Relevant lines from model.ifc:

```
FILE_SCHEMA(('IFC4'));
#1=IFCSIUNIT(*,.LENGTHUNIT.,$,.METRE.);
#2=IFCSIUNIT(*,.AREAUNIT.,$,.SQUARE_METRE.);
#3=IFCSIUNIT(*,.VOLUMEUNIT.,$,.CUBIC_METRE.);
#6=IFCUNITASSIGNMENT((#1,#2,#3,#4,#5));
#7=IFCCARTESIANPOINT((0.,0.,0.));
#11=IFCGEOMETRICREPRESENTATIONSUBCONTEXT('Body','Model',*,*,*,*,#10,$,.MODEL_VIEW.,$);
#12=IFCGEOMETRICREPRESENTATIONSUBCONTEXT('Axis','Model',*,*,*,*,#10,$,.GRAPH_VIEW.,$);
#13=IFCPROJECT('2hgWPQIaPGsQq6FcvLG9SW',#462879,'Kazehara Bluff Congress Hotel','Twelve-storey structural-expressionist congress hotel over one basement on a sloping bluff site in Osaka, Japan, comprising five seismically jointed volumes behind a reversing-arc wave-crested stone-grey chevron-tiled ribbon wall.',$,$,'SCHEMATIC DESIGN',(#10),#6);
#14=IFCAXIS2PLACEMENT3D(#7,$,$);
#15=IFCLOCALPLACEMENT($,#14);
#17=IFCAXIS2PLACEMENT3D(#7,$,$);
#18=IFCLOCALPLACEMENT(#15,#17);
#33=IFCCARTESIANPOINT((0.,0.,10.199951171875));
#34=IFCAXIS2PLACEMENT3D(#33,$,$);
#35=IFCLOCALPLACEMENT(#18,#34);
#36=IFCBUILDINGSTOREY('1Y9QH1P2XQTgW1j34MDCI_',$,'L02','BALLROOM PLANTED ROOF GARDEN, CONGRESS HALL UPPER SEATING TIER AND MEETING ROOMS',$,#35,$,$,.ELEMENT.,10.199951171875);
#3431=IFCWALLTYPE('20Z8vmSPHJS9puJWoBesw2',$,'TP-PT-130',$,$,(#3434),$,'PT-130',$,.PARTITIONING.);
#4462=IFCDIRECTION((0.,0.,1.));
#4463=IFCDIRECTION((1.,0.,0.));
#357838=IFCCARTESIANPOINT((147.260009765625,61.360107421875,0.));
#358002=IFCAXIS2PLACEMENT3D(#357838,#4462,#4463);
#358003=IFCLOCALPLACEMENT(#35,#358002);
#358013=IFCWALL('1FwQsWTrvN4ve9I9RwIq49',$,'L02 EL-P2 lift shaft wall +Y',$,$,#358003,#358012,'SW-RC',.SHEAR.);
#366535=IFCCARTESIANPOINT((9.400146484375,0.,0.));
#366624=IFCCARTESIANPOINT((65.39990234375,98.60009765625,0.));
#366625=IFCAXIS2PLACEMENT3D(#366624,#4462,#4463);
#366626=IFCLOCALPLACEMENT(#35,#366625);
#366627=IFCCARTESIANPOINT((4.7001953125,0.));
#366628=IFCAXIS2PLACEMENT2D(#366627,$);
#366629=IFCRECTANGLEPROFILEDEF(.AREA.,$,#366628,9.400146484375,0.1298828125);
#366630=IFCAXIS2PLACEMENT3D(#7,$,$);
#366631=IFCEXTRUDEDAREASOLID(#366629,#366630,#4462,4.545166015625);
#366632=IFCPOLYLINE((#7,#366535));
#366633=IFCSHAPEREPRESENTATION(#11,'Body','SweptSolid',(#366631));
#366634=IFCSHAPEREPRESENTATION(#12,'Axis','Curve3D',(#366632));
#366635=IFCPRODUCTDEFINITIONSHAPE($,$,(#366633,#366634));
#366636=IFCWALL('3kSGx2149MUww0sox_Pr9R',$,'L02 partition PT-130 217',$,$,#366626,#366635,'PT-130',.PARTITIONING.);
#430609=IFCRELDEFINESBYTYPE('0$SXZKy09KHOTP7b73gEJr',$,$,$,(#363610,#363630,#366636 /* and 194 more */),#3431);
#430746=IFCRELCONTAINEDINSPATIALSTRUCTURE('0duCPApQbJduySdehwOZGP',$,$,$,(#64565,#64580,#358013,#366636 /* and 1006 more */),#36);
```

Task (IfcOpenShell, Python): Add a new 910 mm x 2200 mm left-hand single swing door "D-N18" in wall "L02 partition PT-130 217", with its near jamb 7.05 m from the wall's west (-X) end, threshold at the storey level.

```python
import numpy as np
import ifcopenshell
import ifcopenshell.api.feature
import ifcopenshell.api.geometry
import ifcopenshell.api.root
import ifcopenshell.api.spatial
import ifcopenshell.geom
import ifcopenshell.util.element
import ifcopenshell.util.placement
import ifcopenshell.util.representation
import ifcopenshell.util.shape
import ifcopenshell.util.unit

model = ifcopenshell.open("model.ifc")
unit_scale = ifcopenshell.util.unit.calculate_unit_scale(model)
settings = ifcopenshell.geom.settings()


def volume(element):
    """Net volume in cubic metres, openings subtracted."""
    shape = ifcopenshell.geom.create_shape(settings, element)
    return ifcopenshell.util.shape.get_volume(shape.geometry)


wall = model.by_id(366636)
storey = ifcopenshell.util.element.get_container(wall, ifc_class="IfcBuildingStorey")
context = ifcopenshell.util.representation.get_context(model, "Model", "Body", "MODEL_VIEW")
before = volume(wall)

width, height, from_end, sill = 0.91, 2.2, 7.05, 0.0  # metres

# The wall runs along its own X axis, and the end named is its -X end.
wall_shape = ifcopenshell.geom.create_shape(settings, wall)
x, y, z = ifcopenshell.util.shape.get_vertices(wall_shape.geometry).T
start = x.min() + from_end
face, thickness = float(y.min()), float(y.max() - y.min())
wall_matrix = ifcopenshell.util.placement.get_local_placement(wall.ObjectPlacement)
level = ifcopenshell.util.placement.get_local_placement(storey.ObjectPlacement)[2, 3]


def in_wall(x, y):
    """Placement at x, y metres in the wall's axes, at sill height."""
    matrix = wall_matrix.copy()
    matrix[:, 3] = wall_matrix @ np.array([x / unit_scale, y / unit_scale, 0.0, 1.0])
    matrix[2, 3] = level + sill / unit_scale
    return matrix


# Opening: a box that overshoots both wall faces by 50 mm.
opening = ifcopenshell.api.root.create_entity(model, ifc_class="IfcOpeningElement", predefined_type="OPENING")
box = ifcopenshell.api.geometry.add_wall_representation(
    model, context=context, length=width, height=height, thickness=thickness + 0.1
)
ifcopenshell.api.geometry.assign_representation(model, product=opening, representation=box)
ifcopenshell.api.geometry.edit_object_placement(model, product=opening, matrix=in_wall(start, face - 0.05), is_si=False)
ifcopenshell.api.feature.add_feature(model, feature=opening, element=wall)

door = ifcopenshell.api.root.create_entity(model, ifc_class="IfcDoor", name="D-N18", predefined_type="DOOR")
door.OverallWidth, door.OverallHeight = width / unit_scale, height / unit_scale
door.OperationType = "SINGLE_SWING_LEFT"
body = ifcopenshell.api.geometry.add_door_representation(
    model,
    context=context,
    overall_width=door.OverallWidth,
    overall_height=door.OverallHeight,
    operation_type="SINGLE_SWING_LEFT",
    lining_properties={"LiningDepth": thickness / unit_scale, "ThresholdDepth": thickness / unit_scale},
)
ifcopenshell.api.geometry.assign_representation(model, product=door, representation=body)
ifcopenshell.api.spatial.assign_container(model, products=[door], relating_structure=storey)
ifcopenshell.api.feature.add_filling(model, opening=opening, element=door)

# The lining spans the wall, so the door starts at the wall face.
ifcopenshell.api.geometry.edit_object_placement(model, product=door, matrix=in_wall(start, face), is_si=False)

after = volume(wall)

print(f"wall volume {before:.3f} -> {after:.3f} m3")

model.write("model_updated.ifc")
```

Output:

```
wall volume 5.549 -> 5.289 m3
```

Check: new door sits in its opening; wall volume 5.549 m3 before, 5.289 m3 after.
